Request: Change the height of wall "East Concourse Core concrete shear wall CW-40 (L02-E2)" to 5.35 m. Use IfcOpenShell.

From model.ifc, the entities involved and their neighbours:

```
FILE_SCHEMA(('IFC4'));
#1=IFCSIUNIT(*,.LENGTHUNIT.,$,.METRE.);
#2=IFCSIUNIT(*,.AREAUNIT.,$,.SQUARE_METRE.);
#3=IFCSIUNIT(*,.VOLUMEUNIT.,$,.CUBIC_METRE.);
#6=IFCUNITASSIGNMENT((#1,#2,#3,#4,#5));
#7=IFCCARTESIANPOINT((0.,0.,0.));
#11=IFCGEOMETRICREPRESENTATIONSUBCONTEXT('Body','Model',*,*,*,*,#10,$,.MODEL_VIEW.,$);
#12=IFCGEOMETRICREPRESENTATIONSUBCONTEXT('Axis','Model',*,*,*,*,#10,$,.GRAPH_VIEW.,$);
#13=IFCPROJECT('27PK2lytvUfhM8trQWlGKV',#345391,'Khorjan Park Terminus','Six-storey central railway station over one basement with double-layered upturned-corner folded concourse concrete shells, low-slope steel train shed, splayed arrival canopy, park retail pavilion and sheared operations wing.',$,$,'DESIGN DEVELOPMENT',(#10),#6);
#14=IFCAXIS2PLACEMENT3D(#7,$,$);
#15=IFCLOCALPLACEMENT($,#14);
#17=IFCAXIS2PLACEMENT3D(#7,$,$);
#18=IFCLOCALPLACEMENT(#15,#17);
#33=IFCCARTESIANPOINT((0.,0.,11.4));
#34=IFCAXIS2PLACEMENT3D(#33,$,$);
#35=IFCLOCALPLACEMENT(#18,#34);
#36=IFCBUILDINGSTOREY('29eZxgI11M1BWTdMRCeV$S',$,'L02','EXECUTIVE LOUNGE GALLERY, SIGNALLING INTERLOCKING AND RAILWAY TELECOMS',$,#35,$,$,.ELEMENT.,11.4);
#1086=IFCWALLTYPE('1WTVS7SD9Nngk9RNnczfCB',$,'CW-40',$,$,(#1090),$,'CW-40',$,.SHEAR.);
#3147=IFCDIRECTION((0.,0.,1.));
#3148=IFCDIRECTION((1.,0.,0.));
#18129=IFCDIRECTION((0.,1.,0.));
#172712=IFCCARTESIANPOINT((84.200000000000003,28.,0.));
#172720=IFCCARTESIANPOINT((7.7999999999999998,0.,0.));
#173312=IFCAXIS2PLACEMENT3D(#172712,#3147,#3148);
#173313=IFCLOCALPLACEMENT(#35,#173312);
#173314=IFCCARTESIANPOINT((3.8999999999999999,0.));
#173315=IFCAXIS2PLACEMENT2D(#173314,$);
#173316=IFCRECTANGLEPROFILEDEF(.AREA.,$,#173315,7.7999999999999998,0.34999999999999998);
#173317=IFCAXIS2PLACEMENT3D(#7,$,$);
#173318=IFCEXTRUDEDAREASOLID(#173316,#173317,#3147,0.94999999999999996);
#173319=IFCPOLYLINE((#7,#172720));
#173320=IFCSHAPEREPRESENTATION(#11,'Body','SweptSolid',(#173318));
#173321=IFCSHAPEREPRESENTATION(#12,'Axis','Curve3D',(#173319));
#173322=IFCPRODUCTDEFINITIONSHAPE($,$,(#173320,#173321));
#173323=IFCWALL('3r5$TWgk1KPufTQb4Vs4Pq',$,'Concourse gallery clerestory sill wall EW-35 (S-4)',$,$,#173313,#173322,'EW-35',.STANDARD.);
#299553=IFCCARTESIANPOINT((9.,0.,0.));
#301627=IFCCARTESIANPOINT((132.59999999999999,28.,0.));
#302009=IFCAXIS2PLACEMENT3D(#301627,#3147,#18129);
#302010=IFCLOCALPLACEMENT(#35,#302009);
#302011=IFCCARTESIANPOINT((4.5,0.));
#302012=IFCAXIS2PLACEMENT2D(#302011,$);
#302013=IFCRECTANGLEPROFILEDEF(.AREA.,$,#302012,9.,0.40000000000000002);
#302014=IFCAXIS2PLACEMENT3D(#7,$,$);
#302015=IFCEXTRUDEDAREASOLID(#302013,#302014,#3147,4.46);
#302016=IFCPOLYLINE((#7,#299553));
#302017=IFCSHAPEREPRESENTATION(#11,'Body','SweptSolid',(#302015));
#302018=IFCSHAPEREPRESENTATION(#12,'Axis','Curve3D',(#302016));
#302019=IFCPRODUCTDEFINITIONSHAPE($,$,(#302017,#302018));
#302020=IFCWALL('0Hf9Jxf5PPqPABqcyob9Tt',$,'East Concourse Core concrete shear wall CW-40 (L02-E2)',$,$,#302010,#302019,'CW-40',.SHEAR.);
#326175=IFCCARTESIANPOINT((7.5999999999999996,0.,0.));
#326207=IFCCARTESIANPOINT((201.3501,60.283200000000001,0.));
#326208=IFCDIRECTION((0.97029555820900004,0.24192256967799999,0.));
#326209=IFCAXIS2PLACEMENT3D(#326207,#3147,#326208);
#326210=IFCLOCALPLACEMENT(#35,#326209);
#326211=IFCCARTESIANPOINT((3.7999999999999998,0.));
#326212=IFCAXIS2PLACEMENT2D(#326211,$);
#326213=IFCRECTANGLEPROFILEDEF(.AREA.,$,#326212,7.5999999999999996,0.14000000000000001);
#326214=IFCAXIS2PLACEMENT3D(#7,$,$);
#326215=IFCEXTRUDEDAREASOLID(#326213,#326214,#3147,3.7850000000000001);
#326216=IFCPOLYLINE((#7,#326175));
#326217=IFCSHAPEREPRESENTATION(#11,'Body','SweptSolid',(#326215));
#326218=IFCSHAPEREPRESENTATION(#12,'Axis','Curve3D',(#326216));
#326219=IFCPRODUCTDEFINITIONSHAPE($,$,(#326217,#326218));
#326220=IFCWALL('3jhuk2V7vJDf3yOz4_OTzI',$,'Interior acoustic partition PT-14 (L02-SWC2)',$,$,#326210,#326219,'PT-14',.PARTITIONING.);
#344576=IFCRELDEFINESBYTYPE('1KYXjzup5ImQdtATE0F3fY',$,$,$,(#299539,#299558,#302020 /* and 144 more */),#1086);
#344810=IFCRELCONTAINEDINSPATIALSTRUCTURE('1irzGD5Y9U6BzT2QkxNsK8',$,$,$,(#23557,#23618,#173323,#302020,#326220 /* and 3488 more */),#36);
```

```python
import ifcopenshell
import ifcopenshell.geom
import ifcopenshell.util.representation
import ifcopenshell.util.shape

model = ifcopenshell.open("model.ifc")
settings = ifcopenshell.geom.settings()


def volume(element):
    """Net volume in cubic metres, openings subtracted."""
    shape = ifcopenshell.geom.create_shape(settings, element)
    return ifcopenshell.util.shape.get_volume(shape.geometry)


wall = model.by_id(302020)
before = volume(wall)

body = ifcopenshell.util.representation.get_representation(wall, "Model", "Body")
solid = body.Items[0]
old_height = solid.Depth
solid.Depth = 5.35
after = volume(wall)

print(f"height {old_height:g} -> {solid.Depth:g}, volume {before:.3f} -> {after:.3f} m3")

model.write("model_updated.ifc")
```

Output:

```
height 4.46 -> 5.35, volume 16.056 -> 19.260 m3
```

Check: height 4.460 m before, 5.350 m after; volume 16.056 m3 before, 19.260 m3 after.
